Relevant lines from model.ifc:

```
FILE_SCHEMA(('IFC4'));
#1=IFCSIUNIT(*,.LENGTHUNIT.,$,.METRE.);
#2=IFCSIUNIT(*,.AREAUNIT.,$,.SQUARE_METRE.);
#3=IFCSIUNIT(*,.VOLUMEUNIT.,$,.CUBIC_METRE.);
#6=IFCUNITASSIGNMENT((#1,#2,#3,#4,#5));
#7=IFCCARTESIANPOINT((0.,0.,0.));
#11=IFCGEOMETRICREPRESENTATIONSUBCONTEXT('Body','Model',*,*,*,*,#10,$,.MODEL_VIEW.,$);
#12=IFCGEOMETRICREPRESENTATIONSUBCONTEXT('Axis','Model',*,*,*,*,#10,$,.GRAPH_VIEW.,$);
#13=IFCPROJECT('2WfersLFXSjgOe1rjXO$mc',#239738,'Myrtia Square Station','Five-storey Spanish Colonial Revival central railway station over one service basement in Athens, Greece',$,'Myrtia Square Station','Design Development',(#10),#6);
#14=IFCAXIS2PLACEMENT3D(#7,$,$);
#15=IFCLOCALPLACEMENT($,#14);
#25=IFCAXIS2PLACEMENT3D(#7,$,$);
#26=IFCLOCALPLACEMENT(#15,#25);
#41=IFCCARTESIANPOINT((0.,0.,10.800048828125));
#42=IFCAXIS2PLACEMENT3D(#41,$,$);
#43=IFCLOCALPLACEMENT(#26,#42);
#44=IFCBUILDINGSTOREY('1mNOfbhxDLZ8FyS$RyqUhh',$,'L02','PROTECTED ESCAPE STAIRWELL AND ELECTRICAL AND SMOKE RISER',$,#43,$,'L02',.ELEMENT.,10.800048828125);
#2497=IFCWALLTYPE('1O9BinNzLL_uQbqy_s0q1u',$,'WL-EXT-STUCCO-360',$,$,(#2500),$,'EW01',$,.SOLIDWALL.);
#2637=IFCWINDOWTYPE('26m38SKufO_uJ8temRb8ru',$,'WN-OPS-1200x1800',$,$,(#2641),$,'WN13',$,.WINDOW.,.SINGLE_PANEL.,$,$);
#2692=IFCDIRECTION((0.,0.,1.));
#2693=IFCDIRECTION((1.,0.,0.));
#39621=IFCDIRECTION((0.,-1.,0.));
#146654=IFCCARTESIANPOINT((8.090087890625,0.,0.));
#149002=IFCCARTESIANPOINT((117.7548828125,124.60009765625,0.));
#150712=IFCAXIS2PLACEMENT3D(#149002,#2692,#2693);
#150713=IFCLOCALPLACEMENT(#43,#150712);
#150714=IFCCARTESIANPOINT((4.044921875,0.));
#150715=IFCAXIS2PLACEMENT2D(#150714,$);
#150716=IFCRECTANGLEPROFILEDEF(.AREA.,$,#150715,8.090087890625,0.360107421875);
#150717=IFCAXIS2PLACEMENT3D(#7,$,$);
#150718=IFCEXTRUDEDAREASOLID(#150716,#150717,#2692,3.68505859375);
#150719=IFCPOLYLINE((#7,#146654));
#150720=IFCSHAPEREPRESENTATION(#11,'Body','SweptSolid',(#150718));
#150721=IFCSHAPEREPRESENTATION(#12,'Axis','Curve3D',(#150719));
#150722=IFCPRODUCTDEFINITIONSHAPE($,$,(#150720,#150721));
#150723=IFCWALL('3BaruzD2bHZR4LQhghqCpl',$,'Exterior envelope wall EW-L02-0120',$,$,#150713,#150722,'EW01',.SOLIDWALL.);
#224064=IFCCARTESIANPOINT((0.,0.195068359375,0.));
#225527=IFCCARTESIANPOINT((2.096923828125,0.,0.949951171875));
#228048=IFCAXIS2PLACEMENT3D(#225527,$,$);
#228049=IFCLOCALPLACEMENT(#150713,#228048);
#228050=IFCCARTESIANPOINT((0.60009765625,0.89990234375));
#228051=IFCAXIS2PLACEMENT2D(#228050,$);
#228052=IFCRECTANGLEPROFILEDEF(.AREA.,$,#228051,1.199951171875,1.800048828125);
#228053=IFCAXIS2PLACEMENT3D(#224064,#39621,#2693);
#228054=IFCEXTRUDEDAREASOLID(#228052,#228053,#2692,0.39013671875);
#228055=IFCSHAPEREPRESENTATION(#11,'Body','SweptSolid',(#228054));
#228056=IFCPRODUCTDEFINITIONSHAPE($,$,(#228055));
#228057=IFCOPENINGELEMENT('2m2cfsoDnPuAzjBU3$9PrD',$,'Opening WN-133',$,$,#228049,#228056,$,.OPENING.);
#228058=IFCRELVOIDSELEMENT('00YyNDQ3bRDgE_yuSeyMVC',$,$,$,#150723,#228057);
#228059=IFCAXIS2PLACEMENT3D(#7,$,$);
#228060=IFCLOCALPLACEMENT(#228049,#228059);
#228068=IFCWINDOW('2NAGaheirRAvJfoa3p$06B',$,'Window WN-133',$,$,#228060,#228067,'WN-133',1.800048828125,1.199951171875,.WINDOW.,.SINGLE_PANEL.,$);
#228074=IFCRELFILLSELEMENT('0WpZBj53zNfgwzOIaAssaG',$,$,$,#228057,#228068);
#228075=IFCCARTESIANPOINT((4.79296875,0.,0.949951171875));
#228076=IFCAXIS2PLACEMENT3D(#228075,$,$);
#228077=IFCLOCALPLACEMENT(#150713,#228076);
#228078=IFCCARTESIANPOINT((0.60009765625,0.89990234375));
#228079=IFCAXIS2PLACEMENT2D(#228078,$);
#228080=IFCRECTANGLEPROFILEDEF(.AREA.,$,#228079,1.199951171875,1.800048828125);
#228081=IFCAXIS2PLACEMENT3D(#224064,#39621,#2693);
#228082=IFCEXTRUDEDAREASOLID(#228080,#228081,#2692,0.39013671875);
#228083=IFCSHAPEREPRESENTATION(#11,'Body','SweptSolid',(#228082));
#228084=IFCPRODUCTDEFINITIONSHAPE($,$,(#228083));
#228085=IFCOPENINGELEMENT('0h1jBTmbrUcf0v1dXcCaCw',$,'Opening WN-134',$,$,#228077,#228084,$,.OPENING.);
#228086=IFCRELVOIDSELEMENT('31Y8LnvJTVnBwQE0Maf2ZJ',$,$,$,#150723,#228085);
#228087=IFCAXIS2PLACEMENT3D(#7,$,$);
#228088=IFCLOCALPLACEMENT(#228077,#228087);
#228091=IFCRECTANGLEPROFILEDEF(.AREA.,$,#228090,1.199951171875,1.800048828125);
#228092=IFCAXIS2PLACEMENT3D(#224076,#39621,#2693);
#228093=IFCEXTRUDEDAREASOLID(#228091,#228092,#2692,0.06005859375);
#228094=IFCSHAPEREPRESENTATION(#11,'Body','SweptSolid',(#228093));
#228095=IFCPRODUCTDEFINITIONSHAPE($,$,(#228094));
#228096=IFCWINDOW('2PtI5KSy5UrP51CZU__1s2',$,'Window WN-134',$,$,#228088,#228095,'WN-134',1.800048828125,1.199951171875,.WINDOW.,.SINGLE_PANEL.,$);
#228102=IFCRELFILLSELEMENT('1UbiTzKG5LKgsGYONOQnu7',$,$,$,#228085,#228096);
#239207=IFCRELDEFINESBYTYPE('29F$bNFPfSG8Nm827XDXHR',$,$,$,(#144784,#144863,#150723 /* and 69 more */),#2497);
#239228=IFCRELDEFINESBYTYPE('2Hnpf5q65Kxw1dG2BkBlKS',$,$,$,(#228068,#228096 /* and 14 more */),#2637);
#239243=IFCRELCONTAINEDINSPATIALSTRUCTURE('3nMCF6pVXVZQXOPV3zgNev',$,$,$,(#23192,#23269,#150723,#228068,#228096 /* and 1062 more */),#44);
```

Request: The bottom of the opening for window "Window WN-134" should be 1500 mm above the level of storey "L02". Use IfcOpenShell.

```python
import numpy as np
import ifcopenshell
import ifcopenshell.api.geometry
import ifcopenshell.geom
import ifcopenshell.util.element
import ifcopenshell.util.placement
import ifcopenshell.util.shape
import ifcopenshell.util.unit

model = ifcopenshell.open("model.ifc")
unit_scale = ifcopenshell.util.unit.calculate_unit_scale(model)

window = model.by_guid("2PtI5KSy5UrP51CZU__1s2")
opening = window.FillsVoids[0].RelatingOpeningElement
storey = ifcopenshell.util.element.get_container(window, ifc_class="IfcBuildingStorey")
level = ifcopenshell.util.placement.get_local_placement(storey.ObjectPlacement)[2, 3]

# The opening's origin need not be at the sill, so measure its lowest point.
shape = ifcopenshell.geom.create_shape(ifcopenshell.geom.settings(), opening)
bottom = ifcopenshell.util.shape.get_shape_bottom_elevation(shape, shape.geometry) / unit_scale
dz = level + 1.5 / unit_scale - bottom

shift = np.array([0.0, 0.0, dz])
# The window is placed relative to its opening, so it follows when the opening moves.
matrix = ifcopenshell.util.placement.get_local_placement(opening.ObjectPlacement)
matrix[:3, 3] += shift
ifcopenshell.api.geometry.edit_object_placement(
    model, product=opening, matrix=matrix, is_si=False, should_transform_children=True
)

print(f"moved by {dz * unit_scale:+.3f} m")

model.write("model-out.ifc")
```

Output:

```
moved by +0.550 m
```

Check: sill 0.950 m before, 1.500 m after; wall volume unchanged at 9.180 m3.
